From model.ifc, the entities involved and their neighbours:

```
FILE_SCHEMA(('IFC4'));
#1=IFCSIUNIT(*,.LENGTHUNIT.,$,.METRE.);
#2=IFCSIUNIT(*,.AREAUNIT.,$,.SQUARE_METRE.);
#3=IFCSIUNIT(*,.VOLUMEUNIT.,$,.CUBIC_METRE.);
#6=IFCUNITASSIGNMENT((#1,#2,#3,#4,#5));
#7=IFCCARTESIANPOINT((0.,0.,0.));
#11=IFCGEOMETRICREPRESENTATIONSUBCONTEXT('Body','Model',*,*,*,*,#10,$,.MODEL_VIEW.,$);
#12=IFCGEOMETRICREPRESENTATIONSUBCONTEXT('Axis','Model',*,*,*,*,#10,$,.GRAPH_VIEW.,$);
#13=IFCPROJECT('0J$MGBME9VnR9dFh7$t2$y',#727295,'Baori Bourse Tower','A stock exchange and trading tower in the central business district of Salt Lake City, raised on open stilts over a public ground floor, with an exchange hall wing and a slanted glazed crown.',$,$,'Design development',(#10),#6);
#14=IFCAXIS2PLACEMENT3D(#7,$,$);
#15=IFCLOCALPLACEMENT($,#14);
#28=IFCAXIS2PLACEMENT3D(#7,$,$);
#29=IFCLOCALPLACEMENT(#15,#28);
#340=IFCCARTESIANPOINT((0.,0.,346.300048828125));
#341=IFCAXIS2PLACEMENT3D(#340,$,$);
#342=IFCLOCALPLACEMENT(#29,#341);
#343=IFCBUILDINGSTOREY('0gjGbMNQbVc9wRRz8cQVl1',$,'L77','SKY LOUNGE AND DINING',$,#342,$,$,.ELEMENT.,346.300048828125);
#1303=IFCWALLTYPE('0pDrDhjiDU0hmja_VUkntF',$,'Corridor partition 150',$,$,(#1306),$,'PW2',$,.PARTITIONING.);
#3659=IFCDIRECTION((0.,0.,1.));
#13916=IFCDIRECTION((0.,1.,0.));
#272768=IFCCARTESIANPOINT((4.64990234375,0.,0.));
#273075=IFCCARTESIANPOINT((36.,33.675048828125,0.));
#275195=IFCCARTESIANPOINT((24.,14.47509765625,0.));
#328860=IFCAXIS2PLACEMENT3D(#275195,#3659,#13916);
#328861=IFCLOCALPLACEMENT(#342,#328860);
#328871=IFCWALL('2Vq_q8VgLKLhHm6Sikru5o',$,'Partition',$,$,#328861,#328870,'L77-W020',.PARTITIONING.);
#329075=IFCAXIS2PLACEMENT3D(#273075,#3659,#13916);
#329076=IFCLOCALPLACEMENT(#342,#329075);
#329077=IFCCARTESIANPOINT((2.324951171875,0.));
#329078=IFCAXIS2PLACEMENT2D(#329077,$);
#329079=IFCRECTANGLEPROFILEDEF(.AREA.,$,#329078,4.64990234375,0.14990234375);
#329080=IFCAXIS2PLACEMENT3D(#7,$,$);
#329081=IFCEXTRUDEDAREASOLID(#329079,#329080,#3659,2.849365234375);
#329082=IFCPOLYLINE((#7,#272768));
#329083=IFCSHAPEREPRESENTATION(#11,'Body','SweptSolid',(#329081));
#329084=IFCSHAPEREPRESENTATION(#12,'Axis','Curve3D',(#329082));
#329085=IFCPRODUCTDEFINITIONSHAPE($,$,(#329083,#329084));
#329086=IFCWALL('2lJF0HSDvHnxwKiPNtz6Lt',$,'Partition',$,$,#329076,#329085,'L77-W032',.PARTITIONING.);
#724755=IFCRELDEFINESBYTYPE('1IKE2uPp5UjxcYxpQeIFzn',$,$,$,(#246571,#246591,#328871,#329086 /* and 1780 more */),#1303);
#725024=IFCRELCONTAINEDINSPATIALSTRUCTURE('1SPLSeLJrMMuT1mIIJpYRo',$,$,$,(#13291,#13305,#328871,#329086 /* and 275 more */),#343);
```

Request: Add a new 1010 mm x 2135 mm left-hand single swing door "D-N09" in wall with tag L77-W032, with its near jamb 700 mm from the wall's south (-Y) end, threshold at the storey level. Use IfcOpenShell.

```python
import numpy as np
import ifcopenshell
import ifcopenshell.api.feature
import ifcopenshell.api.geometry
import ifcopenshell.api.root
import ifcopenshell.api.spatial
import ifcopenshell.geom
import ifcopenshell.util.element
import ifcopenshell.util.placement
import ifcopenshell.util.representation
import ifcopenshell.util.shape
import ifcopenshell.util.unit

model = ifcopenshell.open("model.ifc")
unit_scale = ifcopenshell.util.unit.calculate_unit_scale(model)
settings = ifcopenshell.geom.settings()


def volume(element):
    """Net volume in cubic metres, openings subtracted."""
    shape = ifcopenshell.geom.create_shape(settings, element)
    return ifcopenshell.util.shape.get_volume(shape.geometry)


wall = model.by_guid("2lJF0HSDvHnxwKiPNtz6Lt")
storey = ifcopenshell.util.element.get_container(wall, ifc_class="IfcBuildingStorey")
context = ifcopenshell.util.representation.get_context(model, "Model", "Body", "MODEL_VIEW")
before = volume(wall)

width, height, from_end, sill = 1.01, 2.135, 0.7, 0.0  # metres

# The wall runs along its own X axis, and the end named is its -X end.
wall_shape = ifcopenshell.geom.create_shape(settings, wall)
x, y, z = ifcopenshell.util.shape.get_vertices(wall_shape.geometry).T
start = x.min() + from_end
face, thickness = float(y.min()), float(y.max() - y.min())
wall_matrix = ifcopenshell.util.placement.get_local_placement(wall.ObjectPlacement)
level = ifcopenshell.util.placement.get_local_placement(storey.ObjectPlacement)[2, 3]


def in_wall(x, y):
    """Placement at x, y metres in the wall's axes, at sill height."""
    matrix = wall_matrix.copy()
    matrix[:, 3] = wall_matrix @ np.array([x / unit_scale, y / unit_scale, 0.0, 1.0])
    matrix[2, 3] = level + sill / unit_scale
    return matrix


# Opening: a box that overshoots both wall faces by 50 mm.
opening = ifcopenshell.api.root.create_entity(model, ifc_class="IfcOpeningElement", predefined_type="OPENING")
box = ifcopenshell.api.geometry.add_wall_representation(
    model, context=context, length=width, height=height, thickness=thickness + 0.1
)
ifcopenshell.api.geometry.assign_representation(model, product=opening, representation=box)
ifcopenshell.api.geometry.edit_object_placement(model, product=opening, matrix=in_wall(start, face - 0.05), is_si=False)
ifcopenshell.api.feature.add_feature(model, feature=opening, element=wall)

door = ifcopenshell.api.root.create_entity(model, ifc_class="IfcDoor", name="D-N09", predefined_type="DOOR")
door.OverallWidth, door.OverallHeight = width / unit_scale, height / unit_scale
door.OperationType = "SINGLE_SWING_LEFT"
body = ifcopenshell.api.geometry.add_door_representation(
    model,
    context=context,
    overall_width=door.OverallWidth,
    overall_height=door.OverallHeight,
    operation_type="SINGLE_SWING_LEFT",
    lining_properties={"LiningDepth": thickness / unit_scale, "ThresholdDepth": thickness / unit_scale},
)
ifcopenshell.api.geometry.assign_representation(model, product=door, representation=body)
ifcopenshell.api.spatial.assign_container(model, products=[door], relating_structure=storey)
ifcopenshell.api.feature.add_filling(model, opening=opening, element=door)

# The lining spans the wall, so the door starts at the wall face.
ifcopenshell.api.geometry.edit_object_placement(model, product=door, matrix=in_wall(start, face), is_si=False)

after = volume(wall)

print(f"wall volume {before:.3f} -> {after:.3f} m3")

model.write("model_edited.ifc")
```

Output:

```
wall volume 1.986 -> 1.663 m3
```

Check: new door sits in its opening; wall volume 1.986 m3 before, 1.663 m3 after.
